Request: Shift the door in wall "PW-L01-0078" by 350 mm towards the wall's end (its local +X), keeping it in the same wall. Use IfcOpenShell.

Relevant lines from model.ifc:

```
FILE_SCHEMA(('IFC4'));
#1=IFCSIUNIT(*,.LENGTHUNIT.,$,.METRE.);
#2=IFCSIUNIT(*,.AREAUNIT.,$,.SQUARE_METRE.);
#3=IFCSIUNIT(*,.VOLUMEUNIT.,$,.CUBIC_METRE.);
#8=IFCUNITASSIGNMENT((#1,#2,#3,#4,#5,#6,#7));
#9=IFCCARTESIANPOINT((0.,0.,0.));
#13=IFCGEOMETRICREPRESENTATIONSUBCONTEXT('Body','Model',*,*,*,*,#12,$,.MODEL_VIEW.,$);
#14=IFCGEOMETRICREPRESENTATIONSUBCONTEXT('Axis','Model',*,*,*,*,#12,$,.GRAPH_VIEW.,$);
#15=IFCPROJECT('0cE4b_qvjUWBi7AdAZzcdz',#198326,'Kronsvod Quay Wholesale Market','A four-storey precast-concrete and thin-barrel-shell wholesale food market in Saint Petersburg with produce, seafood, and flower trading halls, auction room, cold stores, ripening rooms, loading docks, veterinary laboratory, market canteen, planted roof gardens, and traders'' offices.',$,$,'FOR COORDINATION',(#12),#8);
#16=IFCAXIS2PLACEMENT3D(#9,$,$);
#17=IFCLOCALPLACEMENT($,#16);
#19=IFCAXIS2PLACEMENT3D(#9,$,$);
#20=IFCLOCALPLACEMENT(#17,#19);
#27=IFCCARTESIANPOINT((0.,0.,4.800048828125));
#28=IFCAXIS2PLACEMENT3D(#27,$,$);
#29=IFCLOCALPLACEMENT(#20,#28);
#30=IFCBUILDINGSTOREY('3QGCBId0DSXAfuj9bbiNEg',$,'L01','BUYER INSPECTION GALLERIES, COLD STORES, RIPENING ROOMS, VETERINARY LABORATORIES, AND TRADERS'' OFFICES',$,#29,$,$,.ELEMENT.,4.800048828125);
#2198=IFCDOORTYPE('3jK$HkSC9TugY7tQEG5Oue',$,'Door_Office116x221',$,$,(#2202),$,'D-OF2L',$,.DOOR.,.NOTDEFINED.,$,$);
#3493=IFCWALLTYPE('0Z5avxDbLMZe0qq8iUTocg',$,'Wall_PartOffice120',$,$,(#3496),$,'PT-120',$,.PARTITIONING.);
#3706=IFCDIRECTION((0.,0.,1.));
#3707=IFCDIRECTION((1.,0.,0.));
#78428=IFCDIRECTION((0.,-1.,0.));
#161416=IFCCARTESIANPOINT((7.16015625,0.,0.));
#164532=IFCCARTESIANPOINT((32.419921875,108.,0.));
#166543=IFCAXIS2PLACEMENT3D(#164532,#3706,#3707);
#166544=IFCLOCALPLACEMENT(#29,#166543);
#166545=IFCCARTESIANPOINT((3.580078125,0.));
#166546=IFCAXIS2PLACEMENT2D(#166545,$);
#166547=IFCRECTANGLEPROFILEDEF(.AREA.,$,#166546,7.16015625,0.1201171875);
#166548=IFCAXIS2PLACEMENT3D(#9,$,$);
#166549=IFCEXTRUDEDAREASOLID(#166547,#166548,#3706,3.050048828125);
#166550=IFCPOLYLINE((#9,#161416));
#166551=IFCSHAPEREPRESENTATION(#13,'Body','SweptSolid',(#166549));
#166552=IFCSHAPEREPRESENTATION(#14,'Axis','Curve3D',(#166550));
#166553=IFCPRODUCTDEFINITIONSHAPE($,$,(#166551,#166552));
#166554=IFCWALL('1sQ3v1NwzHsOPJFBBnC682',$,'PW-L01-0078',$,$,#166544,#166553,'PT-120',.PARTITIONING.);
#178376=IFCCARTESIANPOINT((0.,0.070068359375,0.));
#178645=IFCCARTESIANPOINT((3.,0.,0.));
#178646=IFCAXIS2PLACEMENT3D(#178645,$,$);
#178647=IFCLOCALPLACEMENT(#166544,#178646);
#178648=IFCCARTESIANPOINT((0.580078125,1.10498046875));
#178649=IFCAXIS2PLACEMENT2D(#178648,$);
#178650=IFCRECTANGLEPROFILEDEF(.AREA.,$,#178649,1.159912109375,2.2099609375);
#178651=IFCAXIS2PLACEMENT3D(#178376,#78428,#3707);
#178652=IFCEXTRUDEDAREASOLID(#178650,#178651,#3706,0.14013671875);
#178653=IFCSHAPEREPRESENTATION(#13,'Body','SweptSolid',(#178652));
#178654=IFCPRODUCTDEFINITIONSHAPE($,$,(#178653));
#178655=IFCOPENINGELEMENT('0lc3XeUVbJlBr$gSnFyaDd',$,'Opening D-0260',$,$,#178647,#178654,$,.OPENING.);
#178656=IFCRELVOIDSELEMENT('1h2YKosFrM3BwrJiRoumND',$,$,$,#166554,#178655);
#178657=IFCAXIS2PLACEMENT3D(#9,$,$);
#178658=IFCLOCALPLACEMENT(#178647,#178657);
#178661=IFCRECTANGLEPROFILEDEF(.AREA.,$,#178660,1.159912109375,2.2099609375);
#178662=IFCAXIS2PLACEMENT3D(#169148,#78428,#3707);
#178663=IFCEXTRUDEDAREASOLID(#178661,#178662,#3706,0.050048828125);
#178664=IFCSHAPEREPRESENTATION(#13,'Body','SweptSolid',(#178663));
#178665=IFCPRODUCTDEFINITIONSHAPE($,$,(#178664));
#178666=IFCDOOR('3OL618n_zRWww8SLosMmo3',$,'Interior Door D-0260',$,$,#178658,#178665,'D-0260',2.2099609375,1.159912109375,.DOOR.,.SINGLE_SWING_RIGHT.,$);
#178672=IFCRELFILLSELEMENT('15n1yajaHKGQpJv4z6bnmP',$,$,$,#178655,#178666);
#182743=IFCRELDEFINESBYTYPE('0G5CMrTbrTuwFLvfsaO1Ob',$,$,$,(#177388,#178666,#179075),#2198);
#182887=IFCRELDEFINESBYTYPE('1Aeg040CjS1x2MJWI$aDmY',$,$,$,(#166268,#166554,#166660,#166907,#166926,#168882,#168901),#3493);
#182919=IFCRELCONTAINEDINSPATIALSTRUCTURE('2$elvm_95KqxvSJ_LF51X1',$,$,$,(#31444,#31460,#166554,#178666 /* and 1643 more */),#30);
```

```python
import ifcopenshell
import ifcopenshell.api.geometry
import ifcopenshell.util.placement

model = ifcopenshell.open("model.ifc")

door = model.by_id(178666)
opening = door.FillsVoids[0].RelatingOpeningElement
wall = opening.VoidsElements[0].RelatingBuildingElement

wall_matrix = ifcopenshell.util.placement.get_local_placement(wall.ObjectPlacement)
shift = wall_matrix[:3, 0] * 0.35
before = ifcopenshell.util.placement.get_local_placement(door.ObjectPlacement)[:3, 3].copy()

# The door is placed relative to its opening, so it follows when the opening moves.
matrix = ifcopenshell.util.placement.get_local_placement(opening.ObjectPlacement)
matrix[:3, 3] += shift
ifcopenshell.api.geometry.edit_object_placement(
    model, product=opening, matrix=matrix, is_si=False, should_transform_children=True
)

after = ifcopenshell.util.placement.get_local_placement(door.ObjectPlacement)[:3, 3]
print("door moved by", (after - before).round(3) + 0.0)

model.write("model_rev.ifc")
```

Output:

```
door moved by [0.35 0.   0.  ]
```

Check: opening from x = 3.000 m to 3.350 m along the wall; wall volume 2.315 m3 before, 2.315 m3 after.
